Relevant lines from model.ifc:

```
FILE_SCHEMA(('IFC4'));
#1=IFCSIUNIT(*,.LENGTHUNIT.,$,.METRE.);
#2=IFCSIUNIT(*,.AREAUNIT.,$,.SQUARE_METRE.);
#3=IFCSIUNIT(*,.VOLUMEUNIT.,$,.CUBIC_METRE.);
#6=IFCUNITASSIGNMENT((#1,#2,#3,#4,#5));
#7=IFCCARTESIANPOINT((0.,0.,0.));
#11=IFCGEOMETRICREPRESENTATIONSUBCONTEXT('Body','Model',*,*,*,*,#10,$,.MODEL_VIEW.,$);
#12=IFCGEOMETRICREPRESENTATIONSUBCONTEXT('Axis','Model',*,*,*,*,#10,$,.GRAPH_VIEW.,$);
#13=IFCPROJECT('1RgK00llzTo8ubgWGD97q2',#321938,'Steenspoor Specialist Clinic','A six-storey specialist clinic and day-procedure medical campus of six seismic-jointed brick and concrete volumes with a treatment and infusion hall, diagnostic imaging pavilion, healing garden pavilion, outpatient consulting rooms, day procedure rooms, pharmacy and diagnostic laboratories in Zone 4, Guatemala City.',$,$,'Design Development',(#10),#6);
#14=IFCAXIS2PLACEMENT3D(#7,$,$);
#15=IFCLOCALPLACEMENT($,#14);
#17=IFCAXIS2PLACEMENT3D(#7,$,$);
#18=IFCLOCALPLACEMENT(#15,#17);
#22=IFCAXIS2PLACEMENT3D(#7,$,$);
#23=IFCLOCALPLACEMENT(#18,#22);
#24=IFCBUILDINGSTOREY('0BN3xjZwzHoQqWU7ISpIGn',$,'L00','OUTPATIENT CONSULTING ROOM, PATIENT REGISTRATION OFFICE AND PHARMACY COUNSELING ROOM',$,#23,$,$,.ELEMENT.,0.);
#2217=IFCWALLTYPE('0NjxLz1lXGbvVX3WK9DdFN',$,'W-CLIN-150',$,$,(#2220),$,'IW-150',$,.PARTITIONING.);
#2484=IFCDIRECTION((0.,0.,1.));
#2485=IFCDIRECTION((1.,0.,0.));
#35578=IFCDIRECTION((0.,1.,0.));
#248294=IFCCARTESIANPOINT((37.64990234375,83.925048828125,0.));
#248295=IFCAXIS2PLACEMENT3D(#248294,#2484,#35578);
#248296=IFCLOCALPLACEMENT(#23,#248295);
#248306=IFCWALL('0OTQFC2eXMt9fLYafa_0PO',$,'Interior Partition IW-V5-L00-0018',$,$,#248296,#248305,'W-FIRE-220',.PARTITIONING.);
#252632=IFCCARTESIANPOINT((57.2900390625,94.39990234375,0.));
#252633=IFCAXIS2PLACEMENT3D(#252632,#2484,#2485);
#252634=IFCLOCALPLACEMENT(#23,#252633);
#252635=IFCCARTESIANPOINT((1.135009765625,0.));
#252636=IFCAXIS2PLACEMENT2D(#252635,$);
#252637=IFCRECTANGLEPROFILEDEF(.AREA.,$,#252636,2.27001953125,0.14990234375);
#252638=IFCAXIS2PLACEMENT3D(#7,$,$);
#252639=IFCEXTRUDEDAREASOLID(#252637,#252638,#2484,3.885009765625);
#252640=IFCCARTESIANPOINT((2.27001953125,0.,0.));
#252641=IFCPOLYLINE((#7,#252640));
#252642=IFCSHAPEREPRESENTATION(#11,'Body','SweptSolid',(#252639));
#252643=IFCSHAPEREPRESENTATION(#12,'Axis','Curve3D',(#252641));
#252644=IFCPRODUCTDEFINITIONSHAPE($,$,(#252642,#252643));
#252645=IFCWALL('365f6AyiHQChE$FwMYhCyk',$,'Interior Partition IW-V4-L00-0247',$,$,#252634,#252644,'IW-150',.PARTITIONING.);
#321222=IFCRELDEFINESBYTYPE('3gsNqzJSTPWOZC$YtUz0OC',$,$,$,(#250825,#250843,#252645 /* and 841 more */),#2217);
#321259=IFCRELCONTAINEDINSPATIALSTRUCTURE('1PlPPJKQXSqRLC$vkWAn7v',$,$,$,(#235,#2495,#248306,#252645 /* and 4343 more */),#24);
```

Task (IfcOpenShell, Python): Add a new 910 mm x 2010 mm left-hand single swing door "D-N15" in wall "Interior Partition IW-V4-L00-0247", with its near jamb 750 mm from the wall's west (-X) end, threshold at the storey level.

```python
import numpy as np
import ifcopenshell
import ifcopenshell.api.feature
import ifcopenshell.api.geometry
import ifcopenshell.api.root
import ifcopenshell.api.spatial
import ifcopenshell.geom
import ifcopenshell.util.element
import ifcopenshell.util.placement
import ifcopenshell.util.representation
import ifcopenshell.util.shape
import ifcopenshell.util.unit

model = ifcopenshell.open("model.ifc")
unit_scale = ifcopenshell.util.unit.calculate_unit_scale(model)
settings = ifcopenshell.geom.settings()


def volume(element):
    """Net volume in cubic metres, openings subtracted."""
    shape = ifcopenshell.geom.create_shape(settings, element)
    return ifcopenshell.util.shape.get_volume(shape.geometry)


wall = model.by_guid("365f6AyiHQChE$FwMYhCyk")
storey = ifcopenshell.util.element.get_container(wall, ifc_class="IfcBuildingStorey")
context = ifcopenshell.util.representation.get_context(model, "Model", "Body", "MODEL_VIEW")
before = volume(wall)

width, height, from_end, sill = 0.91, 2.01, 0.75, 0.0  # metres

# The wall runs along its own X axis, and the end named is its -X end.
wall_shape = ifcopenshell.geom.create_shape(settings, wall)
x, y, z = ifcopenshell.util.shape.get_vertices(wall_shape.geometry).T
start = x.min() + from_end
face, thickness = float(y.min()), float(y.max() - y.min())
wall_matrix = ifcopenshell.util.placement.get_local_placement(wall.ObjectPlacement)
level = ifcopenshell.util.placement.get_local_placement(storey.ObjectPlacement)[2, 3]


def in_wall(x, y):
    """Placement at x, y metres in the wall's axes, at sill height."""
    matrix = wall_matrix.copy()
    matrix[:, 3] = wall_matrix @ np.array([x / unit_scale, y / unit_scale, 0.0, 1.0])
    matrix[2, 3] = level + sill / unit_scale
    return matrix


# Opening: a box that overshoots both wall faces by 50 mm.
opening = ifcopenshell.api.root.create_entity(model, ifc_class="IfcOpeningElement", predefined_type="OPENING")
box = ifcopenshell.api.geometry.add_wall_representation(
    model, context=context, length=width, height=height, thickness=thickness + 0.1
)
ifcopenshell.api.geometry.assign_representation(model, product=opening, representation=box)
ifcopenshell.api.geometry.edit_object_placement(model, product=opening, matrix=in_wall(start, face - 0.05), is_si=False)
ifcopenshell.api.feature.add_feature(model, feature=opening, element=wall)

door = ifcopenshell.api.root.create_entity(model, ifc_class="IfcDoor", name="D-N15", predefined_type="DOOR")
door.OverallWidth, door.OverallHeight = width / unit_scale, height / unit_scale
door.OperationType = "SINGLE_SWING_LEFT"
body = ifcopenshell.api.geometry.add_door_representation(
    model,
    context=context,
    overall_width=door.OverallWidth,
    overall_height=door.OverallHeight,
    operation_type="SINGLE_SWING_LEFT",
    lining_properties={"LiningDepth": thickness / unit_scale, "ThresholdDepth": thickness / unit_scale},
)
ifcopenshell.api.geometry.assign_representation(model, product=door, representation=body)
ifcopenshell.api.spatial.assign_container(model, products=[door], relating_structure=storey)
ifcopenshell.api.feature.add_filling(model, opening=opening, element=door)

# The lining spans the wall, so the door starts at the wall face.
ifcopenshell.api.geometry.edit_object_placement(model, product=door, matrix=in_wall(start, face), is_si=False)

after = volume(wall)

print(f"wall volume {before:.3f} -> {after:.3f} m3")

model.write("model-out.ifc")
```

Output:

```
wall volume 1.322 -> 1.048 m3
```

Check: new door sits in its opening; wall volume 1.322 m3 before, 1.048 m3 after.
